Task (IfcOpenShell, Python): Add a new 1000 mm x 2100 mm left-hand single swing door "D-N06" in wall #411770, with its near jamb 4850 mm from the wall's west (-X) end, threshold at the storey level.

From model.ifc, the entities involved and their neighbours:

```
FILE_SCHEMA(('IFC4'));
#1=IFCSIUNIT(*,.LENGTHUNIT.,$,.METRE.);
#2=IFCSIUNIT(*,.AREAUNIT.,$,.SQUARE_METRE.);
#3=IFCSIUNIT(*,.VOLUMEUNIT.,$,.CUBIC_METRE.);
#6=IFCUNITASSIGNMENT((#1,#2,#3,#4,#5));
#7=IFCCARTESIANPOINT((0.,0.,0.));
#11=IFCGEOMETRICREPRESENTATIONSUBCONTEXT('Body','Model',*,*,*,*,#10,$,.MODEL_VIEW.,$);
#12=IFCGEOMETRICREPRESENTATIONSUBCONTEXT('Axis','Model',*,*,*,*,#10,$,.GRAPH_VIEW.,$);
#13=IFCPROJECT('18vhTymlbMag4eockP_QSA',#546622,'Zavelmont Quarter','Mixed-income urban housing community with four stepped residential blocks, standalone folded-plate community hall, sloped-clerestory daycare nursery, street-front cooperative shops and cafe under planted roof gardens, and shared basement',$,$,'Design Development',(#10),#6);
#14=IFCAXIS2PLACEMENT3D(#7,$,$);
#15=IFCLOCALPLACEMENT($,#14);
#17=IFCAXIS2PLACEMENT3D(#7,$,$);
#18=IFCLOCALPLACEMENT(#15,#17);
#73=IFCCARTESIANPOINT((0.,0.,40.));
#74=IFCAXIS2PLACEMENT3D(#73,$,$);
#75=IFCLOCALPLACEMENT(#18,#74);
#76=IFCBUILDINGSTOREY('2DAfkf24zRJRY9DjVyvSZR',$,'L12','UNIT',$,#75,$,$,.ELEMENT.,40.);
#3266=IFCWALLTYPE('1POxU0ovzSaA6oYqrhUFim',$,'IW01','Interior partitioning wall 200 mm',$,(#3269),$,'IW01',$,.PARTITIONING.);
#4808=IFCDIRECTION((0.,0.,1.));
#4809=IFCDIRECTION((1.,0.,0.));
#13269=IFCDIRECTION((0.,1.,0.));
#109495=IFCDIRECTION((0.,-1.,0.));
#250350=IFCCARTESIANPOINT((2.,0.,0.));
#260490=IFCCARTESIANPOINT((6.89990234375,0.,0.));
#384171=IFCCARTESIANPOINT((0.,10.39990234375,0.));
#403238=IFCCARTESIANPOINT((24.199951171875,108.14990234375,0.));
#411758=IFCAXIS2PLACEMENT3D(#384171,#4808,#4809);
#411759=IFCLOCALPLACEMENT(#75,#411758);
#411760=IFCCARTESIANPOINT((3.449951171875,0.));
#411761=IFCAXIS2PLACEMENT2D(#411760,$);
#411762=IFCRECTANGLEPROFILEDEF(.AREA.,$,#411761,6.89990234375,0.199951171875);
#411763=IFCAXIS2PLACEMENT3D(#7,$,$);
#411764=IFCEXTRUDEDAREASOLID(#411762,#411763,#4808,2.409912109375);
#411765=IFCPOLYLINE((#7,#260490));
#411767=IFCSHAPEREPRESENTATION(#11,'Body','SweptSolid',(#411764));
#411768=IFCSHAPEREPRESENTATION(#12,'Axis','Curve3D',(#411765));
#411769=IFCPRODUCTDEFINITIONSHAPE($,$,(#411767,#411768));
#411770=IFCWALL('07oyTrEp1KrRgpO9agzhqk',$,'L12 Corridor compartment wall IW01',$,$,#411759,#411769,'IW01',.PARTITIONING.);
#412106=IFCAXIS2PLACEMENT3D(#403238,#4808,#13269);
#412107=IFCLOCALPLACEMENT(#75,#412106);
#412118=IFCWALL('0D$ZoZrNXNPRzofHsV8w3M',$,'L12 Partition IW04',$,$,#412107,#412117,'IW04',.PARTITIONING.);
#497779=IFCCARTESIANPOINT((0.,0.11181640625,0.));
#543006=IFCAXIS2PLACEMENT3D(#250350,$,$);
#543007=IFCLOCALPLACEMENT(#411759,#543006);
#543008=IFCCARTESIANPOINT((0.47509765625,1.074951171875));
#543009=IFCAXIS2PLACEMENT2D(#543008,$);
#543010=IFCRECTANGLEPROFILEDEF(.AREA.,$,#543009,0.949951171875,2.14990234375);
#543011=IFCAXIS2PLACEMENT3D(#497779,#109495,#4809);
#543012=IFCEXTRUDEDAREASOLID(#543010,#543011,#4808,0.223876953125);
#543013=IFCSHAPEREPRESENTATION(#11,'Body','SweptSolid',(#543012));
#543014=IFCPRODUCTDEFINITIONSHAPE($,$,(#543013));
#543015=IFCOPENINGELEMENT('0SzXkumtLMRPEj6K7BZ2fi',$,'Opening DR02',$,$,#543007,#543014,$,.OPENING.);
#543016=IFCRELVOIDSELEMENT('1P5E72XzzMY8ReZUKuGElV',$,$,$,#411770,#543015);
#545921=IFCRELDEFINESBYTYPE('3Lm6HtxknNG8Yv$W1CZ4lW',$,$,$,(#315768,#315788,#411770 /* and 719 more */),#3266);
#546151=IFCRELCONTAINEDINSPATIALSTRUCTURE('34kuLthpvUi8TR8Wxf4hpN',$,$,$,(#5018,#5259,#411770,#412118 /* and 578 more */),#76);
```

```python
import numpy as np
import ifcopenshell
import ifcopenshell.api.feature
import ifcopenshell.api.geometry
import ifcopenshell.api.root
import ifcopenshell.api.spatial
import ifcopenshell.geom
import ifcopenshell.util.element
import ifcopenshell.util.placement
import ifcopenshell.util.representation
import ifcopenshell.util.shape
import ifcopenshell.util.unit

model = ifcopenshell.open("model.ifc")
unit_scale = ifcopenshell.util.unit.calculate_unit_scale(model)
settings = ifcopenshell.geom.settings()


def volume(element):
    """Net volume in cubic metres, openings subtracted."""
    shape = ifcopenshell.geom.create_shape(settings, element)
    return ifcopenshell.util.shape.get_volume(shape.geometry)


wall = model.by_id(411770)
storey = ifcopenshell.util.element.get_container(wall, ifc_class="IfcBuildingStorey")
context = ifcopenshell.util.representation.get_context(model, "Model", "Body", "MODEL_VIEW")
before = volume(wall)

width, height, from_end, sill = 1, 2.1, 4.85, 0.0  # metres

# The wall runs along its own X axis, and the end named is its -X end.
wall_shape = ifcopenshell.geom.create_shape(settings, wall)
x, y, z = ifcopenshell.util.shape.get_vertices(wall_shape.geometry).T
start = x.min() + from_end
face, thickness = float(y.min()), float(y.max() - y.min())
wall_matrix = ifcopenshell.util.placement.get_local_placement(wall.ObjectPlacement)
level = ifcopenshell.util.placement.get_local_placement(storey.ObjectPlacement)[2, 3]


def in_wall(x, y):
    """Placement at x, y metres in the wall's axes, at sill height."""
    matrix = wall_matrix.copy()
    matrix[:, 3] = wall_matrix @ np.array([x / unit_scale, y / unit_scale, 0.0, 1.0])
    matrix[2, 3] = level + sill / unit_scale
    return matrix


# Opening: a box that overshoots both wall faces by 50 mm.
opening = ifcopenshell.api.root.create_entity(model, ifc_class="IfcOpeningElement", predefined_type="OPENING")
box = ifcopenshell.api.geometry.add_wall_representation(
    model, context=context, length=width, height=height, thickness=thickness + 0.1
)
ifcopenshell.api.geometry.assign_representation(model, product=opening, representation=box)
ifcopenshell.api.geometry.edit_object_placement(model, product=opening, matrix=in_wall(start, face - 0.05), is_si=False)
ifcopenshell.api.feature.add_feature(model, feature=opening, element=wall)

door = ifcopenshell.api.root.create_entity(model, ifc_class="IfcDoor", name="D-N06", predefined_type="DOOR")
door.OverallWidth, door.OverallHeight = width / unit_scale, height / unit_scale
door.OperationType = "SINGLE_SWING_LEFT"
body = ifcopenshell.api.geometry.add_door_representation(
    model,
    context=context,
    overall_width=door.OverallWidth,
    overall_height=door.OverallHeight,
    operation_type="SINGLE_SWING_LEFT",
    lining_properties={"LiningDepth": thickness / unit_scale, "ThresholdDepth": thickness / unit_scale},
)
ifcopenshell.api.geometry.assign_representation(model, product=door, representation=body)
ifcopenshell.api.spatial.assign_container(model, products=[door], relating_structure=storey)
ifcopenshell.api.feature.add_filling(model, opening=opening, element=door)

# The lining spans the wall, so the door starts at the wall face.
ifcopenshell.api.geometry.edit_object_placement(model, product=door, matrix=in_wall(start, face), is_si=False)

after = volume(wall)

print(f"wall volume {before:.3f} -> {after:.3f} m3")

model.write("model_updated.ifc")
```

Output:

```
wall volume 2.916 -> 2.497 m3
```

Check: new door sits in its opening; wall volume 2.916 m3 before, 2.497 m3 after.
